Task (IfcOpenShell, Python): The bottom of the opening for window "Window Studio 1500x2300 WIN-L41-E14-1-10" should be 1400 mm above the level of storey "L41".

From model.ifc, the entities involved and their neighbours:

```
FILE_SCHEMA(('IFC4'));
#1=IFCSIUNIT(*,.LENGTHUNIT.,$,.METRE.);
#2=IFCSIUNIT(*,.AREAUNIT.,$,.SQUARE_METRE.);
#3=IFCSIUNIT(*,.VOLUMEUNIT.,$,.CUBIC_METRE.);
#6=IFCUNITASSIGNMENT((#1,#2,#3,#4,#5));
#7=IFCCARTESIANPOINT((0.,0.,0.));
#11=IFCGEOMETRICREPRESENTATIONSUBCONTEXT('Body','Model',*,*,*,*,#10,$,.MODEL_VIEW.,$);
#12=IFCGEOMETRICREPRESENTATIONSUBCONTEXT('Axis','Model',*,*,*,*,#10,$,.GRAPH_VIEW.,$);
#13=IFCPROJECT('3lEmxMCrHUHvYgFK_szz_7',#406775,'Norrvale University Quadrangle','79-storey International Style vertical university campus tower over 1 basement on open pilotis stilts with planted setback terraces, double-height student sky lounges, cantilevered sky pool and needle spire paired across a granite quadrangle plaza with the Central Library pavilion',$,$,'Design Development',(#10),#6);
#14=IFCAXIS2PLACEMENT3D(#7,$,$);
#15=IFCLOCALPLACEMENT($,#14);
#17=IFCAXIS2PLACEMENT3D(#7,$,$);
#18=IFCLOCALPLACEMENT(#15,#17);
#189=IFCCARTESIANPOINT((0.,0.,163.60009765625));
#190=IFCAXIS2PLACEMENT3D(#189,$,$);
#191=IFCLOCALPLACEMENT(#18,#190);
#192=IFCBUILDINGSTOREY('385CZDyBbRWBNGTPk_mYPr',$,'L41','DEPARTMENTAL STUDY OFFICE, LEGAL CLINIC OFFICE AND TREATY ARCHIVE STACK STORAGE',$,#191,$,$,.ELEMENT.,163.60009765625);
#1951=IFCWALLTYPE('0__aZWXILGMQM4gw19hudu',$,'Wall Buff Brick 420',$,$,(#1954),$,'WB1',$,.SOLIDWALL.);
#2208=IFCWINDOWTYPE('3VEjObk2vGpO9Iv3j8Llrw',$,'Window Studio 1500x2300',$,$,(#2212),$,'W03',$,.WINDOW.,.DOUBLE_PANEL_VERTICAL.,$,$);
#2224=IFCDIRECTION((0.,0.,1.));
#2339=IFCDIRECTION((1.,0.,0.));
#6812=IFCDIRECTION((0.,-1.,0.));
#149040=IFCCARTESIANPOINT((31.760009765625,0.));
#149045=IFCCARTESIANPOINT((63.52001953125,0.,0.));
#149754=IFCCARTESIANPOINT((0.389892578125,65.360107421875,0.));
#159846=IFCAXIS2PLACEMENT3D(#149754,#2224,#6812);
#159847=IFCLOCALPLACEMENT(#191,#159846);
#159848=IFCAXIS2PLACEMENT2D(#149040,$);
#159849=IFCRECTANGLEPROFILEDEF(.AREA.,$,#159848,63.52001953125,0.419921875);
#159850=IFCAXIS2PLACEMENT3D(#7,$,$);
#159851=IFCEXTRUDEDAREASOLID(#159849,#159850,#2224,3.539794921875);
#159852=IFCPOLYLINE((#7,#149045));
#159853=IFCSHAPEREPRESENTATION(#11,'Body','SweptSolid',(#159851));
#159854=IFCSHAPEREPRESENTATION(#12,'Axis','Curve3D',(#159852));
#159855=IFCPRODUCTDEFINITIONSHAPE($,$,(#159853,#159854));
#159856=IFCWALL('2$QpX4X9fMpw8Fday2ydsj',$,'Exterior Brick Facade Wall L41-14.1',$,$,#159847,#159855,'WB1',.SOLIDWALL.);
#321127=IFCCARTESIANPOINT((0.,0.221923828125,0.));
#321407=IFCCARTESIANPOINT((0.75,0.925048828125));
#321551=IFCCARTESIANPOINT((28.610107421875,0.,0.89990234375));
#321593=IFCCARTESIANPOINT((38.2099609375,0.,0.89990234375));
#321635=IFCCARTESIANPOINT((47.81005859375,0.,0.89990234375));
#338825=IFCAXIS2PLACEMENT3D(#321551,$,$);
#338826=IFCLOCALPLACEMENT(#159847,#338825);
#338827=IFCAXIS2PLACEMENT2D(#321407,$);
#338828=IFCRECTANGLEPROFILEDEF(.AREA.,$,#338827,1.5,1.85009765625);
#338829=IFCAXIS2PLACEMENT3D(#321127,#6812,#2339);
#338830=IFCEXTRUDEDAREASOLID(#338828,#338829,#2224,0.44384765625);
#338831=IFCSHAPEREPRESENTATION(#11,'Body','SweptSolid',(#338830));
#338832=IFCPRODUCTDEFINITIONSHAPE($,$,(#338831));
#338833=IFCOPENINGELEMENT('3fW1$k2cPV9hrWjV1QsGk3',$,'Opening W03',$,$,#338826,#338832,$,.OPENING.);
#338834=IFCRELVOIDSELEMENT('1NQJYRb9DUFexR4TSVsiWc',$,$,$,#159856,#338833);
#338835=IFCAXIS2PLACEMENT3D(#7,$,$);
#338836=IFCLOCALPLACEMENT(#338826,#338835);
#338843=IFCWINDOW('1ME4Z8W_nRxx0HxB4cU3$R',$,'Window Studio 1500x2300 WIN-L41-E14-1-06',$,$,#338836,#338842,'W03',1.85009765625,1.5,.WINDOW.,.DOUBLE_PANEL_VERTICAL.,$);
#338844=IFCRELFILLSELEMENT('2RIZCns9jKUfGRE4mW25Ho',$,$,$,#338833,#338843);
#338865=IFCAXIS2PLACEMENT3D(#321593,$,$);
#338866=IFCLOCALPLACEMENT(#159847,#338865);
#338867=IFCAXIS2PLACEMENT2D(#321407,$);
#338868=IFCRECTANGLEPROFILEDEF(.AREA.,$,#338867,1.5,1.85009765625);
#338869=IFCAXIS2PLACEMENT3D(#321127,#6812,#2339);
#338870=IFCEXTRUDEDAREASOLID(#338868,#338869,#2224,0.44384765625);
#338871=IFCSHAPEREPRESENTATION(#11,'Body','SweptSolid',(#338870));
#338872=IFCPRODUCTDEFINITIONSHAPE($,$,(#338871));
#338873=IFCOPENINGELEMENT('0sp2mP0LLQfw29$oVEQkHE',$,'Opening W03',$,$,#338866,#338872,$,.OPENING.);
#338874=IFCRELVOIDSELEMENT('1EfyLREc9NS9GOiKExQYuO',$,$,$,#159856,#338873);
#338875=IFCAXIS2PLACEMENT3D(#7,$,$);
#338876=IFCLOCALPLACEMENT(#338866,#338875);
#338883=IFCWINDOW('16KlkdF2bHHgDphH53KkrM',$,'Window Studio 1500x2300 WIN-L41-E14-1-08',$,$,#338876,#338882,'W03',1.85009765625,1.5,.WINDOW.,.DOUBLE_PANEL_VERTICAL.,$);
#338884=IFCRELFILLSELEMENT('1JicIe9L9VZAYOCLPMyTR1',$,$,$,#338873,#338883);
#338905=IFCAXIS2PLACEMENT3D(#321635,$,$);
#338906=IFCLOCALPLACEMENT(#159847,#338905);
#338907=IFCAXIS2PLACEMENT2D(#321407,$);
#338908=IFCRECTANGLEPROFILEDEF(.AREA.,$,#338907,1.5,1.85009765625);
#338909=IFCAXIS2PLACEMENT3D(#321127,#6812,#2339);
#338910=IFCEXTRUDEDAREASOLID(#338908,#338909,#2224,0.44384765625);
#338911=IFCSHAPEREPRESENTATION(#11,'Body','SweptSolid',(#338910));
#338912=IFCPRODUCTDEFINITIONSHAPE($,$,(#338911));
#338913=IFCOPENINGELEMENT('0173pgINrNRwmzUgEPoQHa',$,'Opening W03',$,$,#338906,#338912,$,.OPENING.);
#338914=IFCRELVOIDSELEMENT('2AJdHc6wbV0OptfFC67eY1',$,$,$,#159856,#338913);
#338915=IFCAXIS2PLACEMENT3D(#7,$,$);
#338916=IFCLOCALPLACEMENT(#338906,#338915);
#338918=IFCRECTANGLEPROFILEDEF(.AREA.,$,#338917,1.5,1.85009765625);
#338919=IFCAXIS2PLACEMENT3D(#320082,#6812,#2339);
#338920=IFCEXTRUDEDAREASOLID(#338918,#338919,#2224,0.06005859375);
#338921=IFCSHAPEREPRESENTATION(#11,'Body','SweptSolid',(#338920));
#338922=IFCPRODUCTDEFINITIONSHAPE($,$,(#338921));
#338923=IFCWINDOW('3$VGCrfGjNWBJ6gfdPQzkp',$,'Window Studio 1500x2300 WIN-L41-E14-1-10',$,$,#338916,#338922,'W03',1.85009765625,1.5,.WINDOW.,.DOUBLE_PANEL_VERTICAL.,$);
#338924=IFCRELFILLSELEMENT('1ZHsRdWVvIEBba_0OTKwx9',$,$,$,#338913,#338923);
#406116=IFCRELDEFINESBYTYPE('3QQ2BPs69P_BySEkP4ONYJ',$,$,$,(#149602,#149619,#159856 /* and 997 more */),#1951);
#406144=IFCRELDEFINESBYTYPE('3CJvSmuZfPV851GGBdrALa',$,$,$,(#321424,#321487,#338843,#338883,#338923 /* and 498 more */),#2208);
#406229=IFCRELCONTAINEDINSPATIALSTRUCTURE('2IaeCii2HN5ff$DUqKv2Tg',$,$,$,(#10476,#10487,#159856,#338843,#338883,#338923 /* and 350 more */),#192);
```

```python
import numpy as np
import ifcopenshell
import ifcopenshell.api.geometry
import ifcopenshell.geom
import ifcopenshell.util.element
import ifcopenshell.util.placement
import ifcopenshell.util.shape
import ifcopenshell.util.unit

model = ifcopenshell.open("model.ifc")
unit_scale = ifcopenshell.util.unit.calculate_unit_scale(model)

window = model.by_id(338923)
opening = window.FillsVoids[0].RelatingOpeningElement
storey = ifcopenshell.util.element.get_container(window, ifc_class="IfcBuildingStorey")
level = ifcopenshell.util.placement.get_local_placement(storey.ObjectPlacement)[2, 3]

# The opening's origin need not be at the sill, so measure its lowest point.
shape = ifcopenshell.geom.create_shape(ifcopenshell.geom.settings(), opening)
bottom = ifcopenshell.util.shape.get_shape_bottom_elevation(shape, shape.geometry) / unit_scale
dz = level + 1.4 - bottom

shift = np.array([0.0, 0.0, dz])
# The window is placed relative to its opening, so it follows when the opening moves.
matrix = ifcopenshell.util.placement.get_local_placement(opening.ObjectPlacement)
matrix[:3, 3] += shift
ifcopenshell.api.geometry.edit_object_placement(
    model, product=opening, matrix=matrix, is_si=False, should_transform_children=True
)

print(f"moved by {dz * unit_scale:+.3f} m")

model.write("model_v2.ifc")
```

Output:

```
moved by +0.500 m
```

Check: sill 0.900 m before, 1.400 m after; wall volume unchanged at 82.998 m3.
